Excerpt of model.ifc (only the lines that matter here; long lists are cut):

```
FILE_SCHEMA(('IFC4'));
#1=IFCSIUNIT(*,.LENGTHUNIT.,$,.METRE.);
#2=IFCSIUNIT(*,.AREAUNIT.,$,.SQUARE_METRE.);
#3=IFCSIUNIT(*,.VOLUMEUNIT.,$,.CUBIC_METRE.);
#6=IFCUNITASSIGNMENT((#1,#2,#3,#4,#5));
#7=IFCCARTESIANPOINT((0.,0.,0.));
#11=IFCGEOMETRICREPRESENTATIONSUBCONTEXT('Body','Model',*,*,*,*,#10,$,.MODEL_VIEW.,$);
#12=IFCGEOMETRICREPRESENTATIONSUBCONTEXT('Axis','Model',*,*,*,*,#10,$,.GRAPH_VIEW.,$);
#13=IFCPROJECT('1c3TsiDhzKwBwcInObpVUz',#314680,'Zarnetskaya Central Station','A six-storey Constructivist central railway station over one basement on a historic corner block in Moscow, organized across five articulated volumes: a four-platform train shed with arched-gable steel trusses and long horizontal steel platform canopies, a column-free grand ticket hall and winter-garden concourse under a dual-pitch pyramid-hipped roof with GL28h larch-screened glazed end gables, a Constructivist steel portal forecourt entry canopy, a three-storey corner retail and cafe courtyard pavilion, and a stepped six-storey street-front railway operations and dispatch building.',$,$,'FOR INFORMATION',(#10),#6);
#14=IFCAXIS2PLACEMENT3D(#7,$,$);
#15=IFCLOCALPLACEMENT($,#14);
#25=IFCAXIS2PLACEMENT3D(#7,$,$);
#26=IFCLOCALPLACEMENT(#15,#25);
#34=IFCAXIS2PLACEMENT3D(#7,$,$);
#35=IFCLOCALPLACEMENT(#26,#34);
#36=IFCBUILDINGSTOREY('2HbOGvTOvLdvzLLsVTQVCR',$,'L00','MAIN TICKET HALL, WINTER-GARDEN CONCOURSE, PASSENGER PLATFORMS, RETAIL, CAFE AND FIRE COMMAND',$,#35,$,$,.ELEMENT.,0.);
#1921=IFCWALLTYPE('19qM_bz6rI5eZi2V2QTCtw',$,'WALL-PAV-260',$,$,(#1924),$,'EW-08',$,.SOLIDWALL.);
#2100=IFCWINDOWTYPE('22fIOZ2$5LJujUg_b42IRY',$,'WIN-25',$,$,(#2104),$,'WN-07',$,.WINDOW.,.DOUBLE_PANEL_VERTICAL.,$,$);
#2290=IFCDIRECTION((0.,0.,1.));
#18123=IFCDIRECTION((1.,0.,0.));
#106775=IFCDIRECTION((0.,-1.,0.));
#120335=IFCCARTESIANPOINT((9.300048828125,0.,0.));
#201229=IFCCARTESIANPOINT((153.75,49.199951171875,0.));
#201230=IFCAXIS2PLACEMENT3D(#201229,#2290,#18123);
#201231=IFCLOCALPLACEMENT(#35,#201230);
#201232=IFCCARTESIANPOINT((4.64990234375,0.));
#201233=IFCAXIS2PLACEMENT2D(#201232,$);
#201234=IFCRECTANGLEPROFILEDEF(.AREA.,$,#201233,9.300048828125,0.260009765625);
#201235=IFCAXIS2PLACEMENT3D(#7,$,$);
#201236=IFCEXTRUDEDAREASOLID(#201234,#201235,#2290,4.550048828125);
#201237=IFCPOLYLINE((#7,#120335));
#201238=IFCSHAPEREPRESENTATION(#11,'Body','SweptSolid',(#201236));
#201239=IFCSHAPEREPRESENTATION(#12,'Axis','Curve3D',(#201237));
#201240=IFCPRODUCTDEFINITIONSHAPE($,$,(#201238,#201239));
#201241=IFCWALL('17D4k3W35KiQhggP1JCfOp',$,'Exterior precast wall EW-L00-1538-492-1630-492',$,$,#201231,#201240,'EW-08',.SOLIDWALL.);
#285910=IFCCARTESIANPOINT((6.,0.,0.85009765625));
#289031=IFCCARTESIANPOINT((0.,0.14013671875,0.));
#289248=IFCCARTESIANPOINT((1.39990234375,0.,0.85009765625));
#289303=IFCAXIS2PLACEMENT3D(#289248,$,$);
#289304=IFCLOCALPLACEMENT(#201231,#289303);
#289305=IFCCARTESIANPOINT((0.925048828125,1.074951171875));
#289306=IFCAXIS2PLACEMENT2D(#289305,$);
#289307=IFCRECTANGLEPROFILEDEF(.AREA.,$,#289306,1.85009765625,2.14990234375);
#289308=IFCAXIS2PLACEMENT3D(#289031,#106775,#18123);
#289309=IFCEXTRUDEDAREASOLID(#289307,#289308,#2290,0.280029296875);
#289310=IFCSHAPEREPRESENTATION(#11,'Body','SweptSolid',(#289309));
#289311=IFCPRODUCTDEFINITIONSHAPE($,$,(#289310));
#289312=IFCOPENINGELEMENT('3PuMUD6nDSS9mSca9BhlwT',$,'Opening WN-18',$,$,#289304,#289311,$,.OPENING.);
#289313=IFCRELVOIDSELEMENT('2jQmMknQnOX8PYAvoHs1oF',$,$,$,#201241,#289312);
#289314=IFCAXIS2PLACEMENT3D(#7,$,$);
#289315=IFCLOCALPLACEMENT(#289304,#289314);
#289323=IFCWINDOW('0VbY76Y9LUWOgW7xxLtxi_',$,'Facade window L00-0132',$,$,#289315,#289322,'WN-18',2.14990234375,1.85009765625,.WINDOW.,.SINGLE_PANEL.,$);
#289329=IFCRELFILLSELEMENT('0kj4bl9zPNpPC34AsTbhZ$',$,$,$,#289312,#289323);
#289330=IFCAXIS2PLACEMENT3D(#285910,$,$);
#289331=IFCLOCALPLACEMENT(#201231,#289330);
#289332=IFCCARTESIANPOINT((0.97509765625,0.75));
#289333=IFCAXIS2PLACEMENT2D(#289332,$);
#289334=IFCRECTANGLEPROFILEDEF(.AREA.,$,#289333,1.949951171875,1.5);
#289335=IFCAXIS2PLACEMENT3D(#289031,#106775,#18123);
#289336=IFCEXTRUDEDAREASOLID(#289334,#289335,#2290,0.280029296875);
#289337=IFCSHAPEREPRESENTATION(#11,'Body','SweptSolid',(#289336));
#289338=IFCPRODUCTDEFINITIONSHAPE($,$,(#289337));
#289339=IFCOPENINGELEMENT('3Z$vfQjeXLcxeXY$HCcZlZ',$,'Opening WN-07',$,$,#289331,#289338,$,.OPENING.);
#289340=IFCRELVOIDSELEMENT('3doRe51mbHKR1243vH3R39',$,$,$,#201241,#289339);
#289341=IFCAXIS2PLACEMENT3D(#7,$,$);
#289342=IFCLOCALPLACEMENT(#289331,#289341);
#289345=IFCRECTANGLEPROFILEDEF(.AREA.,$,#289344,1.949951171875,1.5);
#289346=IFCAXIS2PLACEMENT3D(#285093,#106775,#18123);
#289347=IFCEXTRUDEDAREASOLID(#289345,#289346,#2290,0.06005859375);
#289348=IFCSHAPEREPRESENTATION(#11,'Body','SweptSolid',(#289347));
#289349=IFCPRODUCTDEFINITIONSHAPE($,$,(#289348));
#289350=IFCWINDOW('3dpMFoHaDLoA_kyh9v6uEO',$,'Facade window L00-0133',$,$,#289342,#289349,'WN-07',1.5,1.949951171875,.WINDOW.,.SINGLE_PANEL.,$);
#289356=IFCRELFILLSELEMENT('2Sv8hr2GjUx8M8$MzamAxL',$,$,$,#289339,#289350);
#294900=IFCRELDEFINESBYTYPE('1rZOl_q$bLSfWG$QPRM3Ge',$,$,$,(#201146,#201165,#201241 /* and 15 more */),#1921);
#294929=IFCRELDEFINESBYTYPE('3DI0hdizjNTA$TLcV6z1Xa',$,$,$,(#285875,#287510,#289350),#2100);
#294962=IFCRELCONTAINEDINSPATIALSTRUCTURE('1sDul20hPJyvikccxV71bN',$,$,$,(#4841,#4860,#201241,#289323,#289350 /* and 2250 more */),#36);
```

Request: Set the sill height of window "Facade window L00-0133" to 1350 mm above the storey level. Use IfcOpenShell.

```python
import numpy as np
import ifcopenshell
import ifcopenshell.api.geometry
import ifcopenshell.geom
import ifcopenshell.util.element
import ifcopenshell.util.placement
import ifcopenshell.util.shape
import ifcopenshell.util.unit

model = ifcopenshell.open("model.ifc")
unit_scale = ifcopenshell.util.unit.calculate_unit_scale(model)

window = model.by_guid("3dpMFoHaDLoA_kyh9v6uEO")
opening = window.FillsVoids[0].RelatingOpeningElement
storey = ifcopenshell.util.element.get_container(window, ifc_class="IfcBuildingStorey")
level = ifcopenshell.util.placement.get_local_placement(storey.ObjectPlacement)[2, 3]

# The opening's origin need not be at the sill, so measure its lowest point.
shape = ifcopenshell.geom.create_shape(ifcopenshell.geom.settings(), opening)
bottom = ifcopenshell.util.shape.get_shape_bottom_elevation(shape, shape.geometry) / unit_scale
dz = level + 1.35 / unit_scale - bottom

shift = np.array([0.0, 0.0, dz])
# The window is placed relative to its opening, so it follows when the opening moves.
matrix = ifcopenshell.util.placement.get_local_placement(opening.ObjectPlacement)
matrix[:3, 3] += shift
ifcopenshell.api.geometry.edit_object_placement(
    model, product=opening, matrix=matrix, is_si=False, should_transform_children=True
)

print(f"moved by {dz * unit_scale:+.3f} m")

model.write("model_v2.ifc")
```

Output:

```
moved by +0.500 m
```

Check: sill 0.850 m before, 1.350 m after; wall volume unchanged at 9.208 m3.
